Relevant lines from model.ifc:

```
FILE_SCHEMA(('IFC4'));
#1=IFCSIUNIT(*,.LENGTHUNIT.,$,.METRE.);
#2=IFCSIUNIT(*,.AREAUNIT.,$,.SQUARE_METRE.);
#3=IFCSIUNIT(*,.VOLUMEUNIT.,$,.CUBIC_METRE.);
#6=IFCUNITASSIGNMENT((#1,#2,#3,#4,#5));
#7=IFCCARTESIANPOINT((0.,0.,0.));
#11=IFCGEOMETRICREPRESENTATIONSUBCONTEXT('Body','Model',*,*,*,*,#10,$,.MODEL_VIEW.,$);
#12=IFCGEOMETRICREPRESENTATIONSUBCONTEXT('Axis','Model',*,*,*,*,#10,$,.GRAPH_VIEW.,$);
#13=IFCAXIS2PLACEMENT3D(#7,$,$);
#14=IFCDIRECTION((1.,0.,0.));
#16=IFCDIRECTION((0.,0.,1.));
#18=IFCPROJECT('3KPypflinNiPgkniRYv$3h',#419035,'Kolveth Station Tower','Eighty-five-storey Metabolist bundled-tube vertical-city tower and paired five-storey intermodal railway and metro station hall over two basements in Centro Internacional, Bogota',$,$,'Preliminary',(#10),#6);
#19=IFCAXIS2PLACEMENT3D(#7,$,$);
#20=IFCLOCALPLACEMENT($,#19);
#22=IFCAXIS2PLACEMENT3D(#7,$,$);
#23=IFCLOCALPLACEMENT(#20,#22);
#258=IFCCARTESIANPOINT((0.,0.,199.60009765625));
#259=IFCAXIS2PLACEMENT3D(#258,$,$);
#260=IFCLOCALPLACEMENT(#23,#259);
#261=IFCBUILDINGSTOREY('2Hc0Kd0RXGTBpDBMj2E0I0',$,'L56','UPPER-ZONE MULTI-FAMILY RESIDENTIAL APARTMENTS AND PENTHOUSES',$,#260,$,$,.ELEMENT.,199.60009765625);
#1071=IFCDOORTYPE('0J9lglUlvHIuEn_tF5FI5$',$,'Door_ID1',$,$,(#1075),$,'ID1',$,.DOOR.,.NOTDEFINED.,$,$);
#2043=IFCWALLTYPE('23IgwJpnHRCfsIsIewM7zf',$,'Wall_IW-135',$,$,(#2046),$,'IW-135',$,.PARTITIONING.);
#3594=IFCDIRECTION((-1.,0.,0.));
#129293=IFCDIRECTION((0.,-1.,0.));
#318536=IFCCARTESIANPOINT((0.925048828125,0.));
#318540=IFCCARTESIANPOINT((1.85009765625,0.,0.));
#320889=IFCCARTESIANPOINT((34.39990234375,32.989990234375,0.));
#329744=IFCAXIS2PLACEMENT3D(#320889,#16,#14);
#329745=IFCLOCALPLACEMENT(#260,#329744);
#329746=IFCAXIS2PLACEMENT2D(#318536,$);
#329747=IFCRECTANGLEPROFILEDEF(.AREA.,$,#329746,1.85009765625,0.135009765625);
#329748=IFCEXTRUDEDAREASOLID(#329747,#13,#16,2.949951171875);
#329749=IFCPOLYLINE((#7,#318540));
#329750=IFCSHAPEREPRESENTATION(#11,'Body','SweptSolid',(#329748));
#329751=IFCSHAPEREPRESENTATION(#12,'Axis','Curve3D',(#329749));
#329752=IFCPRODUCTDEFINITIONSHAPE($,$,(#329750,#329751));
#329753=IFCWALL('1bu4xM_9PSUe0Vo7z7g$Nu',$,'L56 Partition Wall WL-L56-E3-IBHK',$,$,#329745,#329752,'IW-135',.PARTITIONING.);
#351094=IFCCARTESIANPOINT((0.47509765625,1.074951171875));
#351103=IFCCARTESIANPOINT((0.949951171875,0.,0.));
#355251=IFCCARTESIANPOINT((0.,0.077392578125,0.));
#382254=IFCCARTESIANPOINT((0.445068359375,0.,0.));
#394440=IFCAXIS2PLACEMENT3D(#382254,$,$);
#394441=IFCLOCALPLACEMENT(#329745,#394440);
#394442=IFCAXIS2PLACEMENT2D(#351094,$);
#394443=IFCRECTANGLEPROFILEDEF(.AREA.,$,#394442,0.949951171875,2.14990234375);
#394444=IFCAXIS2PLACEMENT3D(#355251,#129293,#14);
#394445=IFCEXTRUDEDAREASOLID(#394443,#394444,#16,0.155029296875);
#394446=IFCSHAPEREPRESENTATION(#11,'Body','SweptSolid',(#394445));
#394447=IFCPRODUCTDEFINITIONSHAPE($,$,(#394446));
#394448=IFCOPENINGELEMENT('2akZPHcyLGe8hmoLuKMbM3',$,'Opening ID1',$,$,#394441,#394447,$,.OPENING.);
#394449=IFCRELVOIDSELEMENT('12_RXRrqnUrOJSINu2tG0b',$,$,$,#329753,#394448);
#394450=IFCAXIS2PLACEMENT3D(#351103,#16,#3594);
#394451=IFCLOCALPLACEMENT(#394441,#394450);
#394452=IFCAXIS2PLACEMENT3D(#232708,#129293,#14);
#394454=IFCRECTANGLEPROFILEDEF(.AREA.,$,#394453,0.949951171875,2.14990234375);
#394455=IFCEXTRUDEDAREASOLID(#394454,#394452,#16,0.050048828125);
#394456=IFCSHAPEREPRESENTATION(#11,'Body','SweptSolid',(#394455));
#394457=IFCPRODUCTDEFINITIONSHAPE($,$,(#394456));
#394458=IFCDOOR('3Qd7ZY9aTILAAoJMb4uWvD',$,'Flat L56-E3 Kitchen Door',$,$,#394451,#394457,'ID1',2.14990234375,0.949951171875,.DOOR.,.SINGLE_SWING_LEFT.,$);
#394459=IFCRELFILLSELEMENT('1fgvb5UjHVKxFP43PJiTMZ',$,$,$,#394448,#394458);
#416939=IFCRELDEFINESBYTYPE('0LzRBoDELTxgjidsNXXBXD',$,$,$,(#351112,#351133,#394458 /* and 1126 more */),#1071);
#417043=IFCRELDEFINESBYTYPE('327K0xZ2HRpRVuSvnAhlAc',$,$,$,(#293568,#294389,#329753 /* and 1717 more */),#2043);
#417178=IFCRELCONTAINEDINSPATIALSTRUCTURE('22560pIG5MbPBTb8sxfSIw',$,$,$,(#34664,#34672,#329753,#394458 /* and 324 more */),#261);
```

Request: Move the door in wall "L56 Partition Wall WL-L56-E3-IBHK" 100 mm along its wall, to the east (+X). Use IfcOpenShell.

```python
import ifcopenshell
import ifcopenshell.api.geometry
import ifcopenshell.util.placement
import ifcopenshell.util.unit

model = ifcopenshell.open("model.ifc")
unit_scale = ifcopenshell.util.unit.calculate_unit_scale(model)

door = model.by_guid("3Qd7ZY9aTILAAoJMb4uWvD")
opening = door.FillsVoids[0].RelatingOpeningElement
wall = opening.VoidsElements[0].RelatingBuildingElement

wall_matrix = ifcopenshell.util.placement.get_local_placement(wall.ObjectPlacement)
shift = wall_matrix[:3, 0] * 0.1 / unit_scale
before = ifcopenshell.util.placement.get_local_placement(door.ObjectPlacement)[:3, 3].copy()

# The door is placed relative to its opening, so it follows when the opening moves.
matrix = ifcopenshell.util.placement.get_local_placement(opening.ObjectPlacement)
matrix[:3, 3] += shift
ifcopenshell.api.geometry.edit_object_placement(
    model, product=opening, matrix=matrix, is_si=False, should_transform_children=True
)

after = ifcopenshell.util.placement.get_local_placement(door.ObjectPlacement)[:3, 3]
print("door moved by", (after - before).round(3) + 0.0)

model.write("model_rev.ifc")
```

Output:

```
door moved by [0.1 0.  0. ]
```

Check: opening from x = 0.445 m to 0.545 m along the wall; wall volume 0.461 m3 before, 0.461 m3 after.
